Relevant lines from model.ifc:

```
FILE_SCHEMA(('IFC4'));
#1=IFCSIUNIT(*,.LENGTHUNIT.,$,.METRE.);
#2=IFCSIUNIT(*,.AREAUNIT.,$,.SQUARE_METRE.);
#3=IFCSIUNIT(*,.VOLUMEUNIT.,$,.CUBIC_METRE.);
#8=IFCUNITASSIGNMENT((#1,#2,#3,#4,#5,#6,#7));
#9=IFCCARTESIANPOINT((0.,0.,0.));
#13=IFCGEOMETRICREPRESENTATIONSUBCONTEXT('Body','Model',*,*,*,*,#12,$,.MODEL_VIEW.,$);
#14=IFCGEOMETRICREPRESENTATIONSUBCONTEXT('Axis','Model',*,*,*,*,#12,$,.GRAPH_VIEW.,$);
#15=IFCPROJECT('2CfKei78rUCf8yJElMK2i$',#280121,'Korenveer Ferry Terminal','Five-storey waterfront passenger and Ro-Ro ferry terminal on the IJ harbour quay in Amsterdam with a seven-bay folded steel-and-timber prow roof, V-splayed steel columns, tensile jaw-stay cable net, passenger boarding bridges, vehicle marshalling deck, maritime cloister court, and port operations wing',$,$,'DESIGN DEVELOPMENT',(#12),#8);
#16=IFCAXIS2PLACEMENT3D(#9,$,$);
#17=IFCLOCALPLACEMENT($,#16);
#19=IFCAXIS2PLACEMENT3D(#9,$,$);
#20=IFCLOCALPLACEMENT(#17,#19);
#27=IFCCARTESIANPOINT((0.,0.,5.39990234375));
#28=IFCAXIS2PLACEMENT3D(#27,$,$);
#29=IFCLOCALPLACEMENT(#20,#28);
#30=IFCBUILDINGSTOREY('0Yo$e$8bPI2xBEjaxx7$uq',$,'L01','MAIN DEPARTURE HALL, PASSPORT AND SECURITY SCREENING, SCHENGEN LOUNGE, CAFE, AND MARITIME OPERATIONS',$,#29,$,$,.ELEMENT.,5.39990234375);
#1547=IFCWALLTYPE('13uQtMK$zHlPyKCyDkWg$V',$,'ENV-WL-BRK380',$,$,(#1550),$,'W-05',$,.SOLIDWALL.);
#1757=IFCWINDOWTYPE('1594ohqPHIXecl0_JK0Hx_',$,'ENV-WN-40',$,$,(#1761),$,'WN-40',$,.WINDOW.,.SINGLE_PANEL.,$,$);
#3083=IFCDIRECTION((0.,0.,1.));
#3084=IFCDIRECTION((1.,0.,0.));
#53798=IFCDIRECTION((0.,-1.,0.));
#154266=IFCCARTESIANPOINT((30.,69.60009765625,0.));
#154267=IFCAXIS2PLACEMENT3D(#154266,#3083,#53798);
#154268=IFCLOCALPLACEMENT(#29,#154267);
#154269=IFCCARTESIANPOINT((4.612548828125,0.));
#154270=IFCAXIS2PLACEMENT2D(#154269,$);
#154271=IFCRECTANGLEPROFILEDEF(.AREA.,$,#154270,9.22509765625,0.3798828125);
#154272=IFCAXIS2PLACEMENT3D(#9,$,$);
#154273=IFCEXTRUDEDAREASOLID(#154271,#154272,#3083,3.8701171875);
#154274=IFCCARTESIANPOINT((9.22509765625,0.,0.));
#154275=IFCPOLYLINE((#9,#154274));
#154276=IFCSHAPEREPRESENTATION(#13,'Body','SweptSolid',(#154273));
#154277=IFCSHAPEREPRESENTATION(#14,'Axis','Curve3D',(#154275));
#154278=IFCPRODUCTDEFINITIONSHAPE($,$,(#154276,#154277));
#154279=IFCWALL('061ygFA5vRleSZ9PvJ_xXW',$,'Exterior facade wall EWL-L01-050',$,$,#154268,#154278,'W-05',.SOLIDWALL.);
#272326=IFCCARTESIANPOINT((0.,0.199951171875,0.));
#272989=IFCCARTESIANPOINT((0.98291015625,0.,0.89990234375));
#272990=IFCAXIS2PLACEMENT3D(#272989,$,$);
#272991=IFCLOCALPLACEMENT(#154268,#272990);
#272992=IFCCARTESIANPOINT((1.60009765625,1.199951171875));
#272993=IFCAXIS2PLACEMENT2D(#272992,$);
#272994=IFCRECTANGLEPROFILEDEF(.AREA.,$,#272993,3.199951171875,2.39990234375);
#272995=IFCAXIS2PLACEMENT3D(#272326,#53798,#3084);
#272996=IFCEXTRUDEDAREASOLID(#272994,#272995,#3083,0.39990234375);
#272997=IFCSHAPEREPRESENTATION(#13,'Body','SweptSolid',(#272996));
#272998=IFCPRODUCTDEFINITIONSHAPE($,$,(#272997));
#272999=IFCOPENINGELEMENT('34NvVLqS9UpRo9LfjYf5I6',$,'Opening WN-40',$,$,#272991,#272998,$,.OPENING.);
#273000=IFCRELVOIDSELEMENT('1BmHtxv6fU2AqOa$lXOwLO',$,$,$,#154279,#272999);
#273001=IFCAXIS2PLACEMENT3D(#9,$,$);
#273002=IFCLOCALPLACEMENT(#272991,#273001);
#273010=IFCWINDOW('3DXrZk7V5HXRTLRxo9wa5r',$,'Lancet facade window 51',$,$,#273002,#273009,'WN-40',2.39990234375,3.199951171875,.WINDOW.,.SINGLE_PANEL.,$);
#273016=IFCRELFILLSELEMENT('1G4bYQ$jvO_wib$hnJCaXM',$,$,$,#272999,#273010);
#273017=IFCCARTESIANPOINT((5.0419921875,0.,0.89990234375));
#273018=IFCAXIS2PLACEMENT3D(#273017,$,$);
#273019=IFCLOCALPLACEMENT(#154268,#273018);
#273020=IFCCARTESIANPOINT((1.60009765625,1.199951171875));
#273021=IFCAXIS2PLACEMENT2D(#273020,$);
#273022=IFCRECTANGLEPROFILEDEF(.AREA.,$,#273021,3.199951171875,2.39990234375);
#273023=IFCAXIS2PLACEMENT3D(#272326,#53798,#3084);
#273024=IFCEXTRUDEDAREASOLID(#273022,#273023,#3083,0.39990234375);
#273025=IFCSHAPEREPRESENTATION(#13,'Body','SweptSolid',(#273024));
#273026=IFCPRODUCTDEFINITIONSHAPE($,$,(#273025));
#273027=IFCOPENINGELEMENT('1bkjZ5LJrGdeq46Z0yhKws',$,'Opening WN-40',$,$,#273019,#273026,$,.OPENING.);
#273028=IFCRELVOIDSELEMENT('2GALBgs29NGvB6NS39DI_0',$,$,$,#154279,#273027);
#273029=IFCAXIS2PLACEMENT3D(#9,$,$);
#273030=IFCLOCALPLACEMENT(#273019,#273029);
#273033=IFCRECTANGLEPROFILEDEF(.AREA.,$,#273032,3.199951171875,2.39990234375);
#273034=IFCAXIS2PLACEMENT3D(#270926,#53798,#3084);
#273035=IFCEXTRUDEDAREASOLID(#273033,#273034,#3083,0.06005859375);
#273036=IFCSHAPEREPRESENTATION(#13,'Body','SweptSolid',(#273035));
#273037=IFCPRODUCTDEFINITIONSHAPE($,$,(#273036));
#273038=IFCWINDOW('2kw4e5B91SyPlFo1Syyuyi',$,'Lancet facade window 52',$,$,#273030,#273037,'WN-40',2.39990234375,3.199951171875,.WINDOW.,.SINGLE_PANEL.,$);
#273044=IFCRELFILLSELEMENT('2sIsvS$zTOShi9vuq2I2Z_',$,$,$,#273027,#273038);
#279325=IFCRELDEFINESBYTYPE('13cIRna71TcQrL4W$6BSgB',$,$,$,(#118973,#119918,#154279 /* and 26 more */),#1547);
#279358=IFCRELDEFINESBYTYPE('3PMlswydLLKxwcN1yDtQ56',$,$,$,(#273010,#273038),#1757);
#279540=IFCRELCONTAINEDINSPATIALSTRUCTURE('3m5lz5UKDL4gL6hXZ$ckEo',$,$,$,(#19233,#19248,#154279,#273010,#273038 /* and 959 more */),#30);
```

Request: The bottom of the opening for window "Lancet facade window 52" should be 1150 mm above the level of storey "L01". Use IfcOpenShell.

```python
import numpy as np
import ifcopenshell
import ifcopenshell.api.geometry
import ifcopenshell.geom
import ifcopenshell.util.element
import ifcopenshell.util.placement
import ifcopenshell.util.shape
import ifcopenshell.util.unit

model = ifcopenshell.open("model.ifc")
unit_scale = ifcopenshell.util.unit.calculate_unit_scale(model)

window = model.by_guid("2kw4e5B91SyPlFo1Syyuyi")
opening = window.FillsVoids[0].RelatingOpeningElement
storey = ifcopenshell.util.element.get_container(window, ifc_class="IfcBuildingStorey")
level = ifcopenshell.util.placement.get_local_placement(storey.ObjectPlacement)[2, 3]

# The opening's origin need not be at the sill, so measure its lowest point.
shape = ifcopenshell.geom.create_shape(ifcopenshell.geom.settings(), opening)
bottom = ifcopenshell.util.shape.get_shape_bottom_elevation(shape, shape.geometry) / unit_scale
dz = level + 1.15 / unit_scale - bottom

shift = np.array([0.0, 0.0, dz])
# The window is placed relative to its opening, so it follows when the opening moves.
matrix = ifcopenshell.util.placement.get_local_placement(opening.ObjectPlacement)
matrix[:3, 3] += shift
ifcopenshell.api.geometry.edit_object_placement(
    model, product=opening, matrix=matrix, is_si=False, should_transform_children=True
)

print(f"moved by {dz * unit_scale:+.3f} m")

model.write("model_rev.ifc")
```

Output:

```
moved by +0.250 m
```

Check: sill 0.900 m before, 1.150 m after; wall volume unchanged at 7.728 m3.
